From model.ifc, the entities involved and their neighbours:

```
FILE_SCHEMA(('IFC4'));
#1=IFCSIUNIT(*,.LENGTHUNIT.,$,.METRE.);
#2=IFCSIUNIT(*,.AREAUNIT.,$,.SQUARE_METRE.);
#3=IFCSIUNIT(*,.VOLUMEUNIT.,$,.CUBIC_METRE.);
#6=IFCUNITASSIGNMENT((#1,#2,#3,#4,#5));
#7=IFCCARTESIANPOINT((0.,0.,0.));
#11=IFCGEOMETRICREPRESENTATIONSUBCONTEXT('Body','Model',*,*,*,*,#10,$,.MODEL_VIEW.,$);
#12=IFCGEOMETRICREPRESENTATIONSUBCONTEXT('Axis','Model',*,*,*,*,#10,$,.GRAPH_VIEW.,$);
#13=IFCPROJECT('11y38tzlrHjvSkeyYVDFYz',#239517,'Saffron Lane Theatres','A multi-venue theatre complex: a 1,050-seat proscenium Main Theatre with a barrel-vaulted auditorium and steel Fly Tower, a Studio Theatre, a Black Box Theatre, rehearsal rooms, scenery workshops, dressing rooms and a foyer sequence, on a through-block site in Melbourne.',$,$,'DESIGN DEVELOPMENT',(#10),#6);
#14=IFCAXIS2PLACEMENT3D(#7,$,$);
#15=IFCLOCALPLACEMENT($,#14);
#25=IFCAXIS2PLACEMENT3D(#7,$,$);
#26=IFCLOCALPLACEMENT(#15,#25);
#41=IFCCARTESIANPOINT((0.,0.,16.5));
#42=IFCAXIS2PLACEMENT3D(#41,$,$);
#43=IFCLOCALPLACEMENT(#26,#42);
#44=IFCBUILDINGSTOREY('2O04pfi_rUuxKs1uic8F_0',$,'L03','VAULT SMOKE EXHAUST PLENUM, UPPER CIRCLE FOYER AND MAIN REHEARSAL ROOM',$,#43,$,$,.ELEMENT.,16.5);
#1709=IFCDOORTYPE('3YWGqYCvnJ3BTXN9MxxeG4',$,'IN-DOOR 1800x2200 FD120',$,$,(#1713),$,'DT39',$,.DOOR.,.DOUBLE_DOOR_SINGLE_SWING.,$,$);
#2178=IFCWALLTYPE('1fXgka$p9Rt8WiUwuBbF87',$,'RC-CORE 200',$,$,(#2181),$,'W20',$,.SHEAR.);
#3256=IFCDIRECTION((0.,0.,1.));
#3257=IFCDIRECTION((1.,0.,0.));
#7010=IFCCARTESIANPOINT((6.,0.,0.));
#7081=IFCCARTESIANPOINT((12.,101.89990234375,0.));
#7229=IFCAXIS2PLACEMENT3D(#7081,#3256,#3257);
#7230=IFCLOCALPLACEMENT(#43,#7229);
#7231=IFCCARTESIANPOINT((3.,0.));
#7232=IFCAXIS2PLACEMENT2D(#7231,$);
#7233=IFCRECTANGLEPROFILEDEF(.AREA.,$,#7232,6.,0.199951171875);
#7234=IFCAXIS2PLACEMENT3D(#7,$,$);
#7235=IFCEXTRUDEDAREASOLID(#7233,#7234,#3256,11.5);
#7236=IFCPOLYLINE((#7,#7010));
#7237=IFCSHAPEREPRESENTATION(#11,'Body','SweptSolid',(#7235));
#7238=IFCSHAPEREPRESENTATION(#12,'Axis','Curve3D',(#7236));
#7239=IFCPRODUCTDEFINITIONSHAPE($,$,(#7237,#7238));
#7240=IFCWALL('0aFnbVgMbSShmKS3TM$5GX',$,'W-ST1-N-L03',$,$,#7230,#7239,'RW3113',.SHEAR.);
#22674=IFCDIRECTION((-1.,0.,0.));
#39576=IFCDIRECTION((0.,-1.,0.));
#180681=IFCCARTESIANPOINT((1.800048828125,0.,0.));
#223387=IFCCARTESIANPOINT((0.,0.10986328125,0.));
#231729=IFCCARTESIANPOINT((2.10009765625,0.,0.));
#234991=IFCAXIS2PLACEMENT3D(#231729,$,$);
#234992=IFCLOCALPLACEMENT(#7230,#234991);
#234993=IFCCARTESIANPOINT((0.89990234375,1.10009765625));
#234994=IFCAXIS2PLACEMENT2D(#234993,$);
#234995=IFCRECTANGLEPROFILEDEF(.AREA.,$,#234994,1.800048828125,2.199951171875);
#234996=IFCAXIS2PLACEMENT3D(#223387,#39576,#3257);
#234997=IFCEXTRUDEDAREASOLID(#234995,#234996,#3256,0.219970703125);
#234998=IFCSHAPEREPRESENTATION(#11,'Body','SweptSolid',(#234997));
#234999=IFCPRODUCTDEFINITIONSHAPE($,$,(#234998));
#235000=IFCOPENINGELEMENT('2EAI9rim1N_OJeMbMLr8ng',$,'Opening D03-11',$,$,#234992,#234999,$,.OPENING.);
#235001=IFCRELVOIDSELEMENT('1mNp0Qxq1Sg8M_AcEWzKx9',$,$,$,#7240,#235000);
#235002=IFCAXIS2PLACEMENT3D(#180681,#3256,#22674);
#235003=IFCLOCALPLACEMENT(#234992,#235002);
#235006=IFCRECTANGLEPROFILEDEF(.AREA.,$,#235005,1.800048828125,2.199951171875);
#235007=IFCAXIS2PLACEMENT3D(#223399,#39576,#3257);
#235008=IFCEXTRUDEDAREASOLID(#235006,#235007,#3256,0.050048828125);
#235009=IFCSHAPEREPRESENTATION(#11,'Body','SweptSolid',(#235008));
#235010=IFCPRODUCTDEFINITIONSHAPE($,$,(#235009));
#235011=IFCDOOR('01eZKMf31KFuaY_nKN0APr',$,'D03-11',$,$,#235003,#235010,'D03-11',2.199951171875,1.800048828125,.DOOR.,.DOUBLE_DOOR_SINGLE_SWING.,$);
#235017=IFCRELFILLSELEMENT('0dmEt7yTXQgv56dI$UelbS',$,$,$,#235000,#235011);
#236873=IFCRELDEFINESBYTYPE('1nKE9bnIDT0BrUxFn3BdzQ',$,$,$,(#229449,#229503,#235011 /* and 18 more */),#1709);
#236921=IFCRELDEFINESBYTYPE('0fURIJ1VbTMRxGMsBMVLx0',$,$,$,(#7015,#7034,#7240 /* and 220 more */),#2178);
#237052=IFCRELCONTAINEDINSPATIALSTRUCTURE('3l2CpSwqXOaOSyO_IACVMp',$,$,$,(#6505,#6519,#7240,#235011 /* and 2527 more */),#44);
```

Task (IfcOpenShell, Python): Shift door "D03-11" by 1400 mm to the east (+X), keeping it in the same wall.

```python
import ifcopenshell
import ifcopenshell.api.geometry
import ifcopenshell.util.placement
import ifcopenshell.util.unit

model = ifcopenshell.open("model.ifc")
unit_scale = ifcopenshell.util.unit.calculate_unit_scale(model)

door = model.by_guid("01eZKMf31KFuaY_nKN0APr")
opening = door.FillsVoids[0].RelatingOpeningElement
wall = opening.VoidsElements[0].RelatingBuildingElement

wall_matrix = ifcopenshell.util.placement.get_local_placement(wall.ObjectPlacement)
shift = wall_matrix[:3, 0] * 1.4 / unit_scale
before = ifcopenshell.util.placement.get_local_placement(door.ObjectPlacement)[:3, 3].copy()

# The door is placed relative to its opening, so it follows when the opening moves.
matrix = ifcopenshell.util.placement.get_local_placement(opening.ObjectPlacement)
matrix[:3, 3] += shift
ifcopenshell.api.geometry.edit_object_placement(
    model, product=opening, matrix=matrix, is_si=False, should_transform_children=True
)

after = ifcopenshell.util.placement.get_local_placement(door.ObjectPlacement)[:3, 3]
print("door moved by", (after - before).round(3) + 0.0)

model.write("model_v2.ifc")
```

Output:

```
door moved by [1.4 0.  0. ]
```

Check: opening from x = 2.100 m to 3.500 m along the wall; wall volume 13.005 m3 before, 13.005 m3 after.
